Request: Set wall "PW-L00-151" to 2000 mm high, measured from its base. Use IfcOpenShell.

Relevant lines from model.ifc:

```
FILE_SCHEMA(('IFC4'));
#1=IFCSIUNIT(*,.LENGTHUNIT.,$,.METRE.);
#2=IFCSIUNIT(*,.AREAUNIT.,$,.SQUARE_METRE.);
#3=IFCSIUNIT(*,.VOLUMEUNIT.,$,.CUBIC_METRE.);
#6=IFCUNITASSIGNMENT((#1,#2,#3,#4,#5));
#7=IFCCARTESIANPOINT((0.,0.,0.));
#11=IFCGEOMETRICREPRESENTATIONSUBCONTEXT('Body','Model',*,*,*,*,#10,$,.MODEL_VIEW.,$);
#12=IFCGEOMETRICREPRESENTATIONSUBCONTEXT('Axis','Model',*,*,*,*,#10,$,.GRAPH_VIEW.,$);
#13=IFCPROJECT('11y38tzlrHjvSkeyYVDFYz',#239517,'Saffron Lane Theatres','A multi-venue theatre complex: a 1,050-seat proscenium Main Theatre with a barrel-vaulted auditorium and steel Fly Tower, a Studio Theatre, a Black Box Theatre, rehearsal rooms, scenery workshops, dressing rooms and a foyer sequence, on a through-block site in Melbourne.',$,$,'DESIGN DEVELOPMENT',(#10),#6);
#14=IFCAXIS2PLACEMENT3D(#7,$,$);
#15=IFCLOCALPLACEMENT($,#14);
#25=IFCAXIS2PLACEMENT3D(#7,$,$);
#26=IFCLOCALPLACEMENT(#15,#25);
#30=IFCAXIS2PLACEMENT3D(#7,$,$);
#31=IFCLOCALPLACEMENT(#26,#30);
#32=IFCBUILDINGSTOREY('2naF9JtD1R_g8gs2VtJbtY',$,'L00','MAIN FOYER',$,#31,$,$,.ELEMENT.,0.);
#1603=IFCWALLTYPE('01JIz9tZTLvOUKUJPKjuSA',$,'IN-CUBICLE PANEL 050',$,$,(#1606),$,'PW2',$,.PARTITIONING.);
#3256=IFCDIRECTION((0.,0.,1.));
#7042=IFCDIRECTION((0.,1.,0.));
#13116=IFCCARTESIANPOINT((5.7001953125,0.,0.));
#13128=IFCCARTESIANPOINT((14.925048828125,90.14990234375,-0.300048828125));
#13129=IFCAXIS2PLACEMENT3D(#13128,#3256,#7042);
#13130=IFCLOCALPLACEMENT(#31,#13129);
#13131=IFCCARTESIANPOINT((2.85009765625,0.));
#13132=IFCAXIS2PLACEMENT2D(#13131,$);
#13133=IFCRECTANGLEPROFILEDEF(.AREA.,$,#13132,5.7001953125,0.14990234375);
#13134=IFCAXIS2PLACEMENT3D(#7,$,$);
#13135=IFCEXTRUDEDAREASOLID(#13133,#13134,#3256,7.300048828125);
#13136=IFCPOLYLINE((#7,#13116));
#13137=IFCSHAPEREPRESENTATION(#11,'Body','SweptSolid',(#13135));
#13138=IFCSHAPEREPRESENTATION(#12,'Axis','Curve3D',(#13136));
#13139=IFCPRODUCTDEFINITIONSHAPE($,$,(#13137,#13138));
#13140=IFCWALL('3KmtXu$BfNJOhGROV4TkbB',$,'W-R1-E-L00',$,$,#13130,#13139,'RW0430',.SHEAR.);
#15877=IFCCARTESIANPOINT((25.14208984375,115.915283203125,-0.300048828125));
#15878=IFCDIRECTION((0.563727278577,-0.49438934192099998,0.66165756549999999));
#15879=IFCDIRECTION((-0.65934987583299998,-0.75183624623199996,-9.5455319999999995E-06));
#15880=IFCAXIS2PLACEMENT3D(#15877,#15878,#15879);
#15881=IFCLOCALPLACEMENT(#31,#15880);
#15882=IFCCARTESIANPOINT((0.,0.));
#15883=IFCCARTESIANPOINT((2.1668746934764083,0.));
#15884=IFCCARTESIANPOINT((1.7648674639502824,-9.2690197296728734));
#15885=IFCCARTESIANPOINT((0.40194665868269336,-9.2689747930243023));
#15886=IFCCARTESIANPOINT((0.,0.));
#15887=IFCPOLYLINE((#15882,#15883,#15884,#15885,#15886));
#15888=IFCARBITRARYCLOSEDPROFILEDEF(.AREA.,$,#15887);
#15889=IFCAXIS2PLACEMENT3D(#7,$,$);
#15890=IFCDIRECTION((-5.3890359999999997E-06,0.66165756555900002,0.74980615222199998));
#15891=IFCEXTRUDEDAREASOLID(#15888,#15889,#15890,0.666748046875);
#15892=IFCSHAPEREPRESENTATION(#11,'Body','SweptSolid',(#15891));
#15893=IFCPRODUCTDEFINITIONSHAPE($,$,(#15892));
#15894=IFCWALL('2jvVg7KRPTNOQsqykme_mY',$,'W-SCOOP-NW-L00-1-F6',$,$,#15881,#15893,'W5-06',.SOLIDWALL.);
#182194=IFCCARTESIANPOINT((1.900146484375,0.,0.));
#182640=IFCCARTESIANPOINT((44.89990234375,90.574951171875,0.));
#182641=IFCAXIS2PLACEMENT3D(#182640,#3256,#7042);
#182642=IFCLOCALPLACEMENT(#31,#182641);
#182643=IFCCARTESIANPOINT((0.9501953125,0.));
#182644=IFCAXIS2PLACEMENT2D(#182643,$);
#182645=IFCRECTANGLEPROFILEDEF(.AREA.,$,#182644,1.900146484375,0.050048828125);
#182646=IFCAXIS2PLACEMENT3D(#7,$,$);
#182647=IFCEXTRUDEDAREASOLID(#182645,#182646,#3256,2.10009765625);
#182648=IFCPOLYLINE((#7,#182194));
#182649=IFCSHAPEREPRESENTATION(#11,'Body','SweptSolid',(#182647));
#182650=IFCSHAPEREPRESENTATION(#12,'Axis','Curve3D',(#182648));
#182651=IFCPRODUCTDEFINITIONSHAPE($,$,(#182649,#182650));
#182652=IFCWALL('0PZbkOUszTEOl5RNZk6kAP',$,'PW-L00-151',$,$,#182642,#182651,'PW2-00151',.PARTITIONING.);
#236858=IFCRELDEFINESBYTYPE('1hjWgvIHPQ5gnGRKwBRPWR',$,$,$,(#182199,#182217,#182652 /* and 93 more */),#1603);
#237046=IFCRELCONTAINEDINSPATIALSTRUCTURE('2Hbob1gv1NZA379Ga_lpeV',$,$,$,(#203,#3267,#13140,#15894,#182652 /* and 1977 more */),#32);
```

```python
import ifcopenshell
import ifcopenshell.geom
import ifcopenshell.util.representation
import ifcopenshell.util.shape
import ifcopenshell.util.unit

model = ifcopenshell.open("model.ifc")
unit_scale = ifcopenshell.util.unit.calculate_unit_scale(model)
settings = ifcopenshell.geom.settings()


def volume(element):
    """Net volume in cubic metres, openings subtracted."""
    shape = ifcopenshell.geom.create_shape(settings, element)
    return ifcopenshell.util.shape.get_volume(shape.geometry)


wall = model.by_guid("0PZbkOUszTEOl5RNZk6kAP")
before = volume(wall)

body = ifcopenshell.util.representation.get_representation(wall, "Model", "Body")
solid = body.Items[0]
old_height = solid.Depth
solid.Depth = 2 / unit_scale
after = volume(wall)

print(f"height {old_height:g} -> {solid.Depth:g}, volume {before:.3f} -> {after:.3f} m3")

model.write("model_v2.ifc")
```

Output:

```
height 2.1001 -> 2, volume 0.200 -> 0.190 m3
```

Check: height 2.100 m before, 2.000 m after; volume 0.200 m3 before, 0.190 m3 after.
